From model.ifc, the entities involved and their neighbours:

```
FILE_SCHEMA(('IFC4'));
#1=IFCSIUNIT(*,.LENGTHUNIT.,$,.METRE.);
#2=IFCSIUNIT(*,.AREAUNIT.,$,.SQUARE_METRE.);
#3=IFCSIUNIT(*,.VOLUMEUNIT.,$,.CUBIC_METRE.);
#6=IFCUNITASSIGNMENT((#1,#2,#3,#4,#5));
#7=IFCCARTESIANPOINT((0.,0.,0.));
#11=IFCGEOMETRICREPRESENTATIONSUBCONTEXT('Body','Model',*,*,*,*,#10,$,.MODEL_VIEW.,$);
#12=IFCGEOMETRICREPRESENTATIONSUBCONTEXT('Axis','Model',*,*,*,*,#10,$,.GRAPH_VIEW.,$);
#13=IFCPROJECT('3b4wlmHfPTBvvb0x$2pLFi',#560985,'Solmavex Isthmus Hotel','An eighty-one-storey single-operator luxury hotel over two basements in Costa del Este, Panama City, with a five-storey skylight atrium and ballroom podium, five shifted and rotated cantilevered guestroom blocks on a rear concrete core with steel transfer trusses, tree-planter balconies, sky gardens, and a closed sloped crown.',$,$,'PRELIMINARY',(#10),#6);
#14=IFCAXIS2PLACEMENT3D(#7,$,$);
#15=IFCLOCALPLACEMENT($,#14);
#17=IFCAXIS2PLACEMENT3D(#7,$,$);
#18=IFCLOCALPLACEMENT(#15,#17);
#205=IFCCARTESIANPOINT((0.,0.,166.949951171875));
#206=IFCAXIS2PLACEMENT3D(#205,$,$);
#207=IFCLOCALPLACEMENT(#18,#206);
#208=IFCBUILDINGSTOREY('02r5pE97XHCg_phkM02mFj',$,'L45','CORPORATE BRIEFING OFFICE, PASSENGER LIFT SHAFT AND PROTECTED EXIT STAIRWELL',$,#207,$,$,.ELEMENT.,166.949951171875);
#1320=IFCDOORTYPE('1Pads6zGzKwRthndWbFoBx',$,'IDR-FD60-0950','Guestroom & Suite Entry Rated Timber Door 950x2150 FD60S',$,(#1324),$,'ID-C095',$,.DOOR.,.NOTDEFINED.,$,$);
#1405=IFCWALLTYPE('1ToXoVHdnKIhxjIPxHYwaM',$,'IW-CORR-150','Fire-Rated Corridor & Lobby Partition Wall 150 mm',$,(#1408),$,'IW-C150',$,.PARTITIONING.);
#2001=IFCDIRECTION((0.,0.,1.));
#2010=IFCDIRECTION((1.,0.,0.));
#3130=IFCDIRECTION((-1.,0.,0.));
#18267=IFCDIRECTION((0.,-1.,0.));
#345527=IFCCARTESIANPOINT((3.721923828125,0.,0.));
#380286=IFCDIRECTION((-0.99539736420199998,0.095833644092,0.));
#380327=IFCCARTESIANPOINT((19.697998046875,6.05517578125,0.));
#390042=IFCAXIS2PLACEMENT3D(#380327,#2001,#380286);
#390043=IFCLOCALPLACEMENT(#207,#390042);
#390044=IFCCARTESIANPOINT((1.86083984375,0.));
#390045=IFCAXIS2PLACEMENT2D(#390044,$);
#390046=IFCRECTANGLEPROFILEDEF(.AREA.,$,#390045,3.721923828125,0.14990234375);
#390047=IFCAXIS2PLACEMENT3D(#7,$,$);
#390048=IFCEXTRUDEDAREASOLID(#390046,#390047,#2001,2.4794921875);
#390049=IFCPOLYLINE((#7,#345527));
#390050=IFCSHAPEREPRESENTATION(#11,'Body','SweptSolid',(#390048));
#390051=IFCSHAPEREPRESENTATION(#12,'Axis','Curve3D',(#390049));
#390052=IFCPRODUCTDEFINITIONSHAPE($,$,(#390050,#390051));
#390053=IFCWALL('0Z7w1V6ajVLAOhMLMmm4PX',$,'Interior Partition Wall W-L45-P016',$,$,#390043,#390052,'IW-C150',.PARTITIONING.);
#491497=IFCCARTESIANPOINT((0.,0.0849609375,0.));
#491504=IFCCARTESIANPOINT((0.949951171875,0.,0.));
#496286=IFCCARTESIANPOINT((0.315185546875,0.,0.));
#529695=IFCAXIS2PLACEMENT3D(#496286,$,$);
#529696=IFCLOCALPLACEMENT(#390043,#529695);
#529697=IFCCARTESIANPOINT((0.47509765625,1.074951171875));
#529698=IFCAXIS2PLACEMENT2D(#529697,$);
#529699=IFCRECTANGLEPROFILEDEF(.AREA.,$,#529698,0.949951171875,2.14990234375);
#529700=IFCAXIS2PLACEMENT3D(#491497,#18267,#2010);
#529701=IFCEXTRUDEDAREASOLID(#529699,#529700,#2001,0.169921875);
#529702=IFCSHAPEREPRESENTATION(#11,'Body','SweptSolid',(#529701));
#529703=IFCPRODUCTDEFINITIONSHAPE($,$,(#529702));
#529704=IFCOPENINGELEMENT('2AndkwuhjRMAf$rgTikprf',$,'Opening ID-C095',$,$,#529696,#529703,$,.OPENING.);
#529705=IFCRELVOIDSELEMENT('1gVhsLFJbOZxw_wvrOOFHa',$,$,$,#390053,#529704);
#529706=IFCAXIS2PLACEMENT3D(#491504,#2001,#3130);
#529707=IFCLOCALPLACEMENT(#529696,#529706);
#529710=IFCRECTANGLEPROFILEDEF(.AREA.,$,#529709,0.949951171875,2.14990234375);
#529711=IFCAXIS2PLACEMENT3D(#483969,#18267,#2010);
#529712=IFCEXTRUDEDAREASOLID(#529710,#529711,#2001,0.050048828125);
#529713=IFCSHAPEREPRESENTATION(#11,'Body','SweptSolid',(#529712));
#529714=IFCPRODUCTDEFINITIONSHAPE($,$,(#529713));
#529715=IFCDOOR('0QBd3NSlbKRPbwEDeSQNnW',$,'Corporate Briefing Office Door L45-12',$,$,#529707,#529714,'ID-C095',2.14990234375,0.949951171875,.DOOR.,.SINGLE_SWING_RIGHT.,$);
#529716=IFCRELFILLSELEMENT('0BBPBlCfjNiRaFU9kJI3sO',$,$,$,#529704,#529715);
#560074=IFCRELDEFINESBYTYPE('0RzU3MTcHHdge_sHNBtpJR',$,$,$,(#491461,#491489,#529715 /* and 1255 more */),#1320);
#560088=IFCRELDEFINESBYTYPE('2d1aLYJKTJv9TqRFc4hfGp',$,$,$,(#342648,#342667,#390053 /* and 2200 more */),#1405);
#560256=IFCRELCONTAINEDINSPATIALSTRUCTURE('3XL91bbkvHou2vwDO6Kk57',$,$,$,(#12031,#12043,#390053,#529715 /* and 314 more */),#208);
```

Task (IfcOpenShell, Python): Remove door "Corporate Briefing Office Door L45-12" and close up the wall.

```python
import ifcopenshell
import ifcopenshell.api.feature
import ifcopenshell.api.root
import ifcopenshell.geom
import ifcopenshell.util.shape

model = ifcopenshell.open("model.ifc")
settings = ifcopenshell.geom.settings()


def volume(element):
    """Net volume in cubic metres, openings subtracted."""
    shape = ifcopenshell.geom.create_shape(settings, element)
    return ifcopenshell.util.shape.get_volume(shape.geometry)


door = model.by_guid("0QBd3NSlbKRPbwEDeSQNnW")
opening = door.FillsVoids[0].RelatingOpeningElement
wall = opening.VoidsElements[0].RelatingBuildingElement
before = volume(wall)

ifcopenshell.api.root.remove_product(model, product=door)
ifcopenshell.api.feature.remove_feature(model, feature=opening)

after = volume(wall)

print(f"wall volume {before:.3f} -> {after:.3f} m3")

model.write("model_edited.ifc")
```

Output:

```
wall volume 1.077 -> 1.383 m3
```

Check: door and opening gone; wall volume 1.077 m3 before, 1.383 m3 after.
